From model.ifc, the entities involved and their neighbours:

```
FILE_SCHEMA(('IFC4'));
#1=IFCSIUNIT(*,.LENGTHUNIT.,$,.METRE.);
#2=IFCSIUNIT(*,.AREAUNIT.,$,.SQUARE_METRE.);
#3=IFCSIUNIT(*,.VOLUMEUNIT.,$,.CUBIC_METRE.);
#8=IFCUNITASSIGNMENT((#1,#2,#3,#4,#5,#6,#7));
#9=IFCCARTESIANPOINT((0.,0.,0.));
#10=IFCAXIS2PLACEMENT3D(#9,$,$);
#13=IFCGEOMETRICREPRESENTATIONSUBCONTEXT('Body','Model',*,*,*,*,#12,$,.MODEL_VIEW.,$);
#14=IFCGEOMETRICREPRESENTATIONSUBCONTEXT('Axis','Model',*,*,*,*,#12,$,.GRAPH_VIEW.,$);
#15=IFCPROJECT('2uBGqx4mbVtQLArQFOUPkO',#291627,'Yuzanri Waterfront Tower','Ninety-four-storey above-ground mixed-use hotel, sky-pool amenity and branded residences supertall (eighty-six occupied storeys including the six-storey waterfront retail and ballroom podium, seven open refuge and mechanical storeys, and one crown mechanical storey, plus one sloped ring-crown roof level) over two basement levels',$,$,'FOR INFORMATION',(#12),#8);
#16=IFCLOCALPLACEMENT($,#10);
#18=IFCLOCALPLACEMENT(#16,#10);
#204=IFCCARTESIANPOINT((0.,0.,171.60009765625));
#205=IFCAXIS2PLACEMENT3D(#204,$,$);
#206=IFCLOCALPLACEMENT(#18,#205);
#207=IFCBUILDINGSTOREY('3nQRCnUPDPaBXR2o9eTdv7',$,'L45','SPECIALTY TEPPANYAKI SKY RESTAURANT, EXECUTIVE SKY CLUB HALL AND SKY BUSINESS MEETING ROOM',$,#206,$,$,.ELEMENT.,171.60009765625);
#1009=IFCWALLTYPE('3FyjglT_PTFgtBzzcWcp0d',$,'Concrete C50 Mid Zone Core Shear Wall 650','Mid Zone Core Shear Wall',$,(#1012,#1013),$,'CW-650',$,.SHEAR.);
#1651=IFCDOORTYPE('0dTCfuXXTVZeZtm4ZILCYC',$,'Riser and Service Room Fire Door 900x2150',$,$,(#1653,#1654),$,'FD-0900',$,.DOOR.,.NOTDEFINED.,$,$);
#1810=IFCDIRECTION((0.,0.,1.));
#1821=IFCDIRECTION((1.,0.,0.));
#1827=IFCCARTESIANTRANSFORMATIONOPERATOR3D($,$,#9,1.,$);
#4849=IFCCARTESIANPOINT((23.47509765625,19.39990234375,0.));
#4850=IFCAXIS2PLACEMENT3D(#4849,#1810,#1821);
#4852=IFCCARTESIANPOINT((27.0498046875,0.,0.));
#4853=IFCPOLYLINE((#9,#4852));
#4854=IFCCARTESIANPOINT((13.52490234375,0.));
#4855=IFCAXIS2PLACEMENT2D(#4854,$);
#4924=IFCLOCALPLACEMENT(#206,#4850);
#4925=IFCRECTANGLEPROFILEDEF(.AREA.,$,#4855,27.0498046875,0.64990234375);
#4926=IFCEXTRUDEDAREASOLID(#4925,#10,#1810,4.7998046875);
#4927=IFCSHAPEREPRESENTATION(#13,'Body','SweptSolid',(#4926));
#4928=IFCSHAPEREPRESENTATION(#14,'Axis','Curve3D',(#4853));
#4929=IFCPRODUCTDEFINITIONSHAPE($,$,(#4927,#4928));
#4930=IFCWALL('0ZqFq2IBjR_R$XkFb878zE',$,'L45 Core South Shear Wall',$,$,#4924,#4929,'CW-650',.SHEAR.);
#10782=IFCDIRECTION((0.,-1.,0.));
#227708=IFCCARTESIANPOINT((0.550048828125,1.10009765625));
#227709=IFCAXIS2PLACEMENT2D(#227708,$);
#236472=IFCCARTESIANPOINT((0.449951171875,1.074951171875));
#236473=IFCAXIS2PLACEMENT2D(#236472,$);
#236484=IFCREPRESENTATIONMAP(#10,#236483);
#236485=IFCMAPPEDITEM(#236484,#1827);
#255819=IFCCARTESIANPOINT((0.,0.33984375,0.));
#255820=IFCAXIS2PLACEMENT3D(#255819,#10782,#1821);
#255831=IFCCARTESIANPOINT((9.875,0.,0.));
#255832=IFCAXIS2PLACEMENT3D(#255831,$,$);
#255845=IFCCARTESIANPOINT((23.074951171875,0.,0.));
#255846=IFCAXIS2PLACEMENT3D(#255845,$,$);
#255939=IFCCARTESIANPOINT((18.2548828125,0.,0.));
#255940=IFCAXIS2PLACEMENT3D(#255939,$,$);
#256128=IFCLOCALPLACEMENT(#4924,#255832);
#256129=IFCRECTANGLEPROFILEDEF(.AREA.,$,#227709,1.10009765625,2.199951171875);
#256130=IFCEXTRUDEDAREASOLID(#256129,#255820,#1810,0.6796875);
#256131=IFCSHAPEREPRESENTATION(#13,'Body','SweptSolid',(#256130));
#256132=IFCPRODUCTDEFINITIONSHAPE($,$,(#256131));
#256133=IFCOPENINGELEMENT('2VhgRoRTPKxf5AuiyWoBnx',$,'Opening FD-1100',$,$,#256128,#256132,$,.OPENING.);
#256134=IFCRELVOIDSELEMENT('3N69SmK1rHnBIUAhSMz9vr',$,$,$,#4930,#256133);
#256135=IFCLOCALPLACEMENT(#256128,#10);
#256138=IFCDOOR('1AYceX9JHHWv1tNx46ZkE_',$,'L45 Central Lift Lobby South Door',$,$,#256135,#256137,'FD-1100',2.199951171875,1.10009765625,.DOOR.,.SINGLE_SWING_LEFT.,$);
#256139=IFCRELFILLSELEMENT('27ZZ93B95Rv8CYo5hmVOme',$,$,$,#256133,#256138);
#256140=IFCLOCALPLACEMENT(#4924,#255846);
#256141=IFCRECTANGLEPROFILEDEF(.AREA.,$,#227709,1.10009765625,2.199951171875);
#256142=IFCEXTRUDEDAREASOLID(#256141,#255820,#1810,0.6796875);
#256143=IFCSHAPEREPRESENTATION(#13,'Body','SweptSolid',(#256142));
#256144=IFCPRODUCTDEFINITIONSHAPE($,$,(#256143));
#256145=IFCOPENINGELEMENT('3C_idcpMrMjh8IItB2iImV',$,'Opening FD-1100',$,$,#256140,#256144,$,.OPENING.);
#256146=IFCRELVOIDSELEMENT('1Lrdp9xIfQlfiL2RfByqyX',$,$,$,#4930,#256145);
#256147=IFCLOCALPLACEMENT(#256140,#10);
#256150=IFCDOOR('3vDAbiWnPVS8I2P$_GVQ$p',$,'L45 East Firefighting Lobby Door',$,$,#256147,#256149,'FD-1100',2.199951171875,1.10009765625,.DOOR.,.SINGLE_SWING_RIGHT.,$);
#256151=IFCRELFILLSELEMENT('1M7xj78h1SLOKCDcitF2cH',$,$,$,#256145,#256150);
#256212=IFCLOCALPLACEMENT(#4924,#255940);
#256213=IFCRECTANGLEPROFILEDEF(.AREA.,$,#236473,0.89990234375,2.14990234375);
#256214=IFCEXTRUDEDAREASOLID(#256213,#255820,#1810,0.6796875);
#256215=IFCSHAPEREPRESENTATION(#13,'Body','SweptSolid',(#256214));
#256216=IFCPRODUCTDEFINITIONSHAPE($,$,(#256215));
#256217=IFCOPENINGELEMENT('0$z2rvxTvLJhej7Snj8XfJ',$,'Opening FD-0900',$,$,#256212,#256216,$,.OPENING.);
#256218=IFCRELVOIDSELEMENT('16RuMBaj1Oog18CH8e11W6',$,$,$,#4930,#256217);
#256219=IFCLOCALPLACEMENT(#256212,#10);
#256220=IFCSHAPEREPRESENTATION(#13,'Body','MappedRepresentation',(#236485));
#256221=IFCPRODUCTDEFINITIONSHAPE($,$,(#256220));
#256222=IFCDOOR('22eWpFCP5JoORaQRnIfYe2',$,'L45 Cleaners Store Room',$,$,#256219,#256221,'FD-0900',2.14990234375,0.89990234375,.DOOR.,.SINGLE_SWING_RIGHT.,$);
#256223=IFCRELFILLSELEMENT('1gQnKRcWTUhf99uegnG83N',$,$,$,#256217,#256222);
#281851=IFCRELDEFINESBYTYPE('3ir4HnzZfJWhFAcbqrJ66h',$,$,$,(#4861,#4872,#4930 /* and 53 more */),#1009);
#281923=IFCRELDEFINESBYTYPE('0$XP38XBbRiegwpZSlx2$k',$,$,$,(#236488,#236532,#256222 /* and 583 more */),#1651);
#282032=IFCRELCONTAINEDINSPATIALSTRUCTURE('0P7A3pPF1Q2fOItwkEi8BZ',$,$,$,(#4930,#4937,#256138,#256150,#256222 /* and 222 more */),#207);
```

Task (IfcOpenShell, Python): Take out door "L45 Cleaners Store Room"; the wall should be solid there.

```python
import ifcopenshell
import ifcopenshell.api.feature
import ifcopenshell.api.root
import ifcopenshell.geom
import ifcopenshell.util.shape

model = ifcopenshell.open("model.ifc")
settings = ifcopenshell.geom.settings()


def volume(element):
    """Net volume in cubic metres, openings subtracted."""
    shape = ifcopenshell.geom.create_shape(settings, element)
    return ifcopenshell.util.shape.get_volume(shape.geometry)


door = model.by_id(256222)
opening = door.FillsVoids[0].RelatingOpeningElement
wall = opening.VoidsElements[0].RelatingBuildingElement
before = volume(wall)

ifcopenshell.api.root.remove_product(model, product=door)
ifcopenshell.api.feature.remove_feature(model, feature=opening)

after = volume(wall)

print(f"wall volume {before:.3f} -> {after:.3f} m3")

model.write("model_edited.ifc")
```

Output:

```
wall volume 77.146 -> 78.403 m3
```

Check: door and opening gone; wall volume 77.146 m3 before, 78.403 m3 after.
